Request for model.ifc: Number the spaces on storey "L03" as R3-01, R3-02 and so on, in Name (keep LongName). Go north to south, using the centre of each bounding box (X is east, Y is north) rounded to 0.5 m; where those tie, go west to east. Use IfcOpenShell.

First a look at what the model holds.

```python
import ifcopenshell
import ifcopenshell.util.element
import ifcopenshell.util.placement

model = ifcopenshell.open("model.ifc")
print(model.schema)
storey = next(s for s in model.by_type("IfcBuildingStorey") if s.Name == "L03")
spaces = [e for e in ifcopenshell.util.element.get_decomposition(storey) if e.is_a("IfcSpace")]
for e in sorted(spaces, key=lambda e: e.id()):
    origin = ifcopenshell.util.placement.get_local_placement(e.ObjectPlacement)[:3, 3]
    print(e.id(), e.Name, e.LongName, origin.round(2) + 0.0, sep=" | ")
```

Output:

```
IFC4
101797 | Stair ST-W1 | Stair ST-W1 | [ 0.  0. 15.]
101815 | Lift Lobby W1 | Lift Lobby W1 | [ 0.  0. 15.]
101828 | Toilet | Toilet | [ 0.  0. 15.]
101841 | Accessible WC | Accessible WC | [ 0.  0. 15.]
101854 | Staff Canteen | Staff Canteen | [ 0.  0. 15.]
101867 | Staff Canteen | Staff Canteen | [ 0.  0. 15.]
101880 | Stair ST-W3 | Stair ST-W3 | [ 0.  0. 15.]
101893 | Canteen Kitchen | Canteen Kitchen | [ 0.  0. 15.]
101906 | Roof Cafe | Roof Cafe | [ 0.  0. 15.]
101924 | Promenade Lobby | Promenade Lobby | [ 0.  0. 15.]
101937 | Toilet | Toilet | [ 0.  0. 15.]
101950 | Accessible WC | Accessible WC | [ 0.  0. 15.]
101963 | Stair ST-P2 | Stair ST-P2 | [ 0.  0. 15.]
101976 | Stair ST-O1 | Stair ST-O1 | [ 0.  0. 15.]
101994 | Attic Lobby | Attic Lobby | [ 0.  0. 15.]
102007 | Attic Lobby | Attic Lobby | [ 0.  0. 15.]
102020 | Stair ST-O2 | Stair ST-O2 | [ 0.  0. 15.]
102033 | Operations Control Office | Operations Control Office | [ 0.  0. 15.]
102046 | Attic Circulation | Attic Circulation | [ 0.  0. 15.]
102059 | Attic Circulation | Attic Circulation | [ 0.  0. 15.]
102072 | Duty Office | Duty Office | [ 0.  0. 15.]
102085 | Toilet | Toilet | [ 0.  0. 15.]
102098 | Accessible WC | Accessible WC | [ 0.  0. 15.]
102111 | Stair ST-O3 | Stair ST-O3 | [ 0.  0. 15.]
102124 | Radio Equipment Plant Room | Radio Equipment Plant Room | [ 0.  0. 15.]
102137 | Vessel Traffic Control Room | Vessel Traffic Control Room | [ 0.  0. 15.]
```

```python
import ifcopenshell
import ifcopenshell.geom
import ifcopenshell.util.element
import ifcopenshell.util.shape

model = ifcopenshell.open("model.ifc")
settings = ifcopenshell.geom.settings()
settings.set("use-world-coords", True)


def centre(element):
    shape = ifcopenshell.geom.create_shape(settings, element)
    return ifcopenshell.util.shape.get_bbox_centroid(shape.geometry)


storey = next(s for s in model.by_type("IfcBuildingStorey") if s.Name == "L03")
spaces = [e for e in ifcopenshell.util.element.get_decomposition(storey) if e.is_a("IfcSpace")]

# Insertion points can sit at a corner or the storey origin, so sort by the geometry (in metres).
centres = {e: centre(e) for e in spaces}
spaces.sort(key=lambda e: (-round(centres[e][1] / 0.5), centres[e][0]))

for i, e in enumerate(spaces, start=1):
    number = f"R3-{i:02d}"
    e.Name = number
    print(e.id(), number)

model.write("model_edited.ifc")
```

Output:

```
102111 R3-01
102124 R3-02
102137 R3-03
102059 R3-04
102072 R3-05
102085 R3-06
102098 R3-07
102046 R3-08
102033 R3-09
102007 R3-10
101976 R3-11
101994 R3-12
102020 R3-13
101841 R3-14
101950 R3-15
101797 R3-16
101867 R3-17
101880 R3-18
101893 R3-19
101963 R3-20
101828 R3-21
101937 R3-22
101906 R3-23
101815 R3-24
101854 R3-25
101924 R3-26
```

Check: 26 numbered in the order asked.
